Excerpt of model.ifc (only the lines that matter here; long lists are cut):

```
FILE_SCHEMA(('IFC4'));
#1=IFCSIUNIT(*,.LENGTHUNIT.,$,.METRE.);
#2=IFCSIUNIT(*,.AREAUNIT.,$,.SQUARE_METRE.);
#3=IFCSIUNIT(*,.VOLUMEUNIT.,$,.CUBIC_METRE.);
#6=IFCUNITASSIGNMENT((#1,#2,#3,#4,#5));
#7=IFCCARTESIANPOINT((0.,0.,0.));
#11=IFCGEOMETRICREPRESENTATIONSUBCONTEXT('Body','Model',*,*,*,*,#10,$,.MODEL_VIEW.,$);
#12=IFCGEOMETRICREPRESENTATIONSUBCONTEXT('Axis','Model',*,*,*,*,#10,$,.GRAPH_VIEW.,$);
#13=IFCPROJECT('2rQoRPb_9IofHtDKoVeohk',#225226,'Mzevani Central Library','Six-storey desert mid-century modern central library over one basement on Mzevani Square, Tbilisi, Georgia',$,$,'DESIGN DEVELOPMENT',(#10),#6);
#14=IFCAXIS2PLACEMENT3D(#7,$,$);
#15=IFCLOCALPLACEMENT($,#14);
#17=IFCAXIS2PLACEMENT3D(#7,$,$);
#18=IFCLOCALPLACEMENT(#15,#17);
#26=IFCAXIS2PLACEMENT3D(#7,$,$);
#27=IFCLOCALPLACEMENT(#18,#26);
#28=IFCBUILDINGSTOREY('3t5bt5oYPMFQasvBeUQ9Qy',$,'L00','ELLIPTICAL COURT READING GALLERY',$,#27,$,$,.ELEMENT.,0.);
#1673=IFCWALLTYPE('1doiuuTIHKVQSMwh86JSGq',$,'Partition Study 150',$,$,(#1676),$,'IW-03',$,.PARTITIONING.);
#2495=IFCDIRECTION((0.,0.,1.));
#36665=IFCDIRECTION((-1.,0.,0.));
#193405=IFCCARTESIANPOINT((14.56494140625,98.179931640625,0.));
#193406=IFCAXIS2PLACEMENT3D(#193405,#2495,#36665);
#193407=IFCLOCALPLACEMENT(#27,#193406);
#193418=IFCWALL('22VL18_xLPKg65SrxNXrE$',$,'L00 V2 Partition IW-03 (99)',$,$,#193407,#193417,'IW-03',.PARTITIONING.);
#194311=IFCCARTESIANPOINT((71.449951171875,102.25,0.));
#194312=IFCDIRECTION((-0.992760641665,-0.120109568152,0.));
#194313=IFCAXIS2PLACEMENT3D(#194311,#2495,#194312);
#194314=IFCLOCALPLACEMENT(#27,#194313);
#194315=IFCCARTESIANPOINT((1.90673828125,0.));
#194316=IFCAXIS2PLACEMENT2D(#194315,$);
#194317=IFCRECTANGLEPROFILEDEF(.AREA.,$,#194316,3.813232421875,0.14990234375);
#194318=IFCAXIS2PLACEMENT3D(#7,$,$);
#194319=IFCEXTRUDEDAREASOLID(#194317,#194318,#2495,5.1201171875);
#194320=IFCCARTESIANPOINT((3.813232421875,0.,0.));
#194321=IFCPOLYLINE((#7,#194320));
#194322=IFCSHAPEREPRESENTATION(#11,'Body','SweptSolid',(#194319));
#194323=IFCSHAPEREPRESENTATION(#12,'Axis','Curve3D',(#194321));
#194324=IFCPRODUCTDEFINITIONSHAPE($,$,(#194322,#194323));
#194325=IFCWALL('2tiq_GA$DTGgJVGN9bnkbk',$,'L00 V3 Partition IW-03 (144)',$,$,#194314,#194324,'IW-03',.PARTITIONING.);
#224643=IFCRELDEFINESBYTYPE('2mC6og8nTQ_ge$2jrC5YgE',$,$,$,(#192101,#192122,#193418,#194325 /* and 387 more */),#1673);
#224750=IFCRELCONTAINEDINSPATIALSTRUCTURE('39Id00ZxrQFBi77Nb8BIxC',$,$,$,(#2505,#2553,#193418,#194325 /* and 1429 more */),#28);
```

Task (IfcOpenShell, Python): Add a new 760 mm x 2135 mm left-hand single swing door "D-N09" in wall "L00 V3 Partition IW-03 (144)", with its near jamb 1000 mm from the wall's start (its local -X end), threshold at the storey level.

```python
import numpy as np
import ifcopenshell
import ifcopenshell.api.feature
import ifcopenshell.api.geometry
import ifcopenshell.api.root
import ifcopenshell.api.spatial
import ifcopenshell.geom
import ifcopenshell.util.element
import ifcopenshell.util.placement
import ifcopenshell.util.representation
import ifcopenshell.util.shape
import ifcopenshell.util.unit

model = ifcopenshell.open("model.ifc")
unit_scale = ifcopenshell.util.unit.calculate_unit_scale(model)
settings = ifcopenshell.geom.settings()


def volume(element):
    """Net volume in cubic metres, openings subtracted."""
    shape = ifcopenshell.geom.create_shape(settings, element)
    return ifcopenshell.util.shape.get_volume(shape.geometry)


wall = model.by_id(194325)
storey = ifcopenshell.util.element.get_container(wall, ifc_class="IfcBuildingStorey")
context = ifcopenshell.util.representation.get_context(model, "Model", "Body", "MODEL_VIEW")
before = volume(wall)

width, height, from_end, sill = 0.76, 2.135, 1, 0.0  # metres

# The wall runs along its own X axis, and the end named is its -X end.
wall_shape = ifcopenshell.geom.create_shape(settings, wall)
x, y, z = ifcopenshell.util.shape.get_vertices(wall_shape.geometry).T
start = x.min() + from_end
face, thickness = float(y.min()), float(y.max() - y.min())
wall_matrix = ifcopenshell.util.placement.get_local_placement(wall.ObjectPlacement)
level = ifcopenshell.util.placement.get_local_placement(storey.ObjectPlacement)[2, 3]


def in_wall(x, y):
    """Placement at x, y metres in the wall's axes, at sill height."""
    matrix = wall_matrix.copy()
    matrix[:, 3] = wall_matrix @ np.array([x / unit_scale, y / unit_scale, 0.0, 1.0])
    matrix[2, 3] = level + sill / unit_scale
    return matrix


# Opening: a box that overshoots both wall faces by 50 mm.
opening = ifcopenshell.api.root.create_entity(model, ifc_class="IfcOpeningElement", predefined_type="OPENING")
box = ifcopenshell.api.geometry.add_wall_representation(
    model, context=context, length=width, height=height, thickness=thickness + 0.1
)
ifcopenshell.api.geometry.assign_representation(model, product=opening, representation=box)
ifcopenshell.api.geometry.edit_object_placement(model, product=opening, matrix=in_wall(start, face - 0.05), is_si=False)
ifcopenshell.api.feature.add_feature(model, feature=opening, element=wall)

door = ifcopenshell.api.root.create_entity(model, ifc_class="IfcDoor", name="D-N09", predefined_type="DOOR")
door.OverallWidth, door.OverallHeight = width / unit_scale, height / unit_scale
door.OperationType = "SINGLE_SWING_LEFT"
body = ifcopenshell.api.geometry.add_door_representation(
    model,
    context=context,
    overall_width=door.OverallWidth,
    overall_height=door.OverallHeight,
    operation_type="SINGLE_SWING_LEFT",
    lining_properties={"LiningDepth": thickness / unit_scale, "ThresholdDepth": thickness / unit_scale},
)
ifcopenshell.api.geometry.assign_representation(model, product=door, representation=body)
ifcopenshell.api.spatial.assign_container(model, products=[door], relating_structure=storey)
ifcopenshell.api.feature.add_filling(model, opening=opening, element=door)

# The lining spans the wall, so the door starts at the wall face.
ifcopenshell.api.geometry.edit_object_placement(model, product=door, matrix=in_wall(start, face), is_si=False)

after = volume(wall)

print(f"wall volume {before:.3f} -> {after:.3f} m3")

model.write("model_rev.ifc")
```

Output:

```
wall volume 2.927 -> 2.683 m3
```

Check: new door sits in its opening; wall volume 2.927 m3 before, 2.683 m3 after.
